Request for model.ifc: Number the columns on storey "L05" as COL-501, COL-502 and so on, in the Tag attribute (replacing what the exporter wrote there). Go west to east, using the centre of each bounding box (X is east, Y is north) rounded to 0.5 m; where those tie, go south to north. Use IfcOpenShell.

First a look at what the model holds.

```python
import ifcopenshell
import ifcopenshell.util.element
import ifcopenshell.util.placement

model = ifcopenshell.open("model.ifc")
print(model.schema)
storey = next(s for s in model.by_type("IfcBuildingStorey") if s.Name == "L05")
columns = [e for e in ifcopenshell.util.element.get_decomposition(storey) if e.is_a("IfcColumn")]
for e in sorted(columns, key=lambda e: e.id()):
    origin = ifcopenshell.util.placement.get_local_placement(e.ObjectPlacement)[:3, 3]
    print(e.id(), e.Tag, e.Name, origin.round(2) + 0.0, sep=" | ")
```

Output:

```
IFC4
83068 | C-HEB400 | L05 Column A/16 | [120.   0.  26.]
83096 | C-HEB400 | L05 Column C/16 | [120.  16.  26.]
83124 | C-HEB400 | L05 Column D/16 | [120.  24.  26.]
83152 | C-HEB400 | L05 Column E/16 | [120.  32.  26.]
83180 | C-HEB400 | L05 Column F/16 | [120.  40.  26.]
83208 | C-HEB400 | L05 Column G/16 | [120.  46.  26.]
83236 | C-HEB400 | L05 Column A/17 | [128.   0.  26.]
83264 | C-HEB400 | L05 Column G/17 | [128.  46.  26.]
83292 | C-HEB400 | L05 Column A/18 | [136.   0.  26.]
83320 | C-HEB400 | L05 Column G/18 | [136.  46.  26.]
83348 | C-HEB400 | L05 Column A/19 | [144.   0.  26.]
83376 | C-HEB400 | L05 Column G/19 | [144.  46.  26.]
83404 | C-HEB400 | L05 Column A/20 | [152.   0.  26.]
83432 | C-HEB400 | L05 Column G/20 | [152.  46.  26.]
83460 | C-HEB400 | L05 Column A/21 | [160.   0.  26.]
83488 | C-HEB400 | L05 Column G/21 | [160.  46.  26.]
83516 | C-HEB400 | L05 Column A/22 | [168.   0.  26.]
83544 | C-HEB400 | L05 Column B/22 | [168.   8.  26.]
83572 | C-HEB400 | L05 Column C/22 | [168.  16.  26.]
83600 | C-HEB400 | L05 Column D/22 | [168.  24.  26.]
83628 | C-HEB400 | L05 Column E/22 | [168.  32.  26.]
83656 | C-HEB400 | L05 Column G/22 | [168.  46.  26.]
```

```python
import ifcopenshell
import ifcopenshell.geom
import ifcopenshell.util.element
import ifcopenshell.util.shape

model = ifcopenshell.open("model.ifc")
settings = ifcopenshell.geom.settings()
settings.set("use-world-coords", True)


def centre(element):
    shape = ifcopenshell.geom.create_shape(settings, element)
    return ifcopenshell.util.shape.get_bbox_centroid(shape.geometry)


storey = next(s for s in model.by_type("IfcBuildingStorey") if s.Name == "L05")
columns = [e for e in ifcopenshell.util.element.get_decomposition(storey) if e.is_a("IfcColumn")]

# Insertion points can sit at a corner or the storey origin, so sort by the geometry (in metres).
centres = {e: centre(e) for e in columns}
columns.sort(key=lambda e: (round(centres[e][0] / 0.5), centres[e][1]))

for i, e in enumerate(columns, start=1):
    number = f"COL-5{i:02d}"
    e.Tag = number
    print(e.id(), number)

model.write("model_edited.ifc")
```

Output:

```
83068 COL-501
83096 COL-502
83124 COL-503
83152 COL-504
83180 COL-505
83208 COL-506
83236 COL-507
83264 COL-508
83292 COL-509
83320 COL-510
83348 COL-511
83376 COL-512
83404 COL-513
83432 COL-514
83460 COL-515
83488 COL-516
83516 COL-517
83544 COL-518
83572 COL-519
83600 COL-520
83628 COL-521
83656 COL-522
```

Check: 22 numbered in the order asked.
